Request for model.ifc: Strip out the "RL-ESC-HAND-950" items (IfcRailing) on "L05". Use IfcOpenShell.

First a look at what the model holds.

```python
import ifcopenshell
import ifcopenshell.util.element

model = ifcopenshell.open("model.ifc")
print(model.schema)
storey = next(s for s in model.by_type("IfcBuildingStorey") if s.Name == "L05")
railings = [e for e in ifcopenshell.util.element.get_decomposition(storey) if e.is_a("IfcRailing")]
seen = {}
for e in railings:
    element_type = ifcopenshell.util.element.get_type(e)
    name = element_type.Name if element_type not in (None, e) else None
    seen[name] = seen.get(name, 0) + 1
for name, count in sorted(seen.items(), key=str):
    print(count, "x", name)
```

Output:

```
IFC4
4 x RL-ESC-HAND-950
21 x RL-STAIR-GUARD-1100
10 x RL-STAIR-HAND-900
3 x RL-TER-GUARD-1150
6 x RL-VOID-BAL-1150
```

```python
import ifcopenshell
import ifcopenshell.api.root
import ifcopenshell.util.element

model = ifcopenshell.open("model.ifc")

storey = next(s for s in model.by_type("IfcBuildingStorey") if s.Name == "L05")
railings = [e for e in ifcopenshell.util.element.get_decomposition(storey) if e.is_a("IfcRailing")]
targets = [e for e in railings if (t := ifcopenshell.util.element.get_type(e)) not in (None, e) and t.Name == "RL-ESC-HAND-950"]

for e in targets:
    ifcopenshell.api.root.remove_product(model, product=e)
print(len(targets), "removed")

model.write("model_v2.ifc")
```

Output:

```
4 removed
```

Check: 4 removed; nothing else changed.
